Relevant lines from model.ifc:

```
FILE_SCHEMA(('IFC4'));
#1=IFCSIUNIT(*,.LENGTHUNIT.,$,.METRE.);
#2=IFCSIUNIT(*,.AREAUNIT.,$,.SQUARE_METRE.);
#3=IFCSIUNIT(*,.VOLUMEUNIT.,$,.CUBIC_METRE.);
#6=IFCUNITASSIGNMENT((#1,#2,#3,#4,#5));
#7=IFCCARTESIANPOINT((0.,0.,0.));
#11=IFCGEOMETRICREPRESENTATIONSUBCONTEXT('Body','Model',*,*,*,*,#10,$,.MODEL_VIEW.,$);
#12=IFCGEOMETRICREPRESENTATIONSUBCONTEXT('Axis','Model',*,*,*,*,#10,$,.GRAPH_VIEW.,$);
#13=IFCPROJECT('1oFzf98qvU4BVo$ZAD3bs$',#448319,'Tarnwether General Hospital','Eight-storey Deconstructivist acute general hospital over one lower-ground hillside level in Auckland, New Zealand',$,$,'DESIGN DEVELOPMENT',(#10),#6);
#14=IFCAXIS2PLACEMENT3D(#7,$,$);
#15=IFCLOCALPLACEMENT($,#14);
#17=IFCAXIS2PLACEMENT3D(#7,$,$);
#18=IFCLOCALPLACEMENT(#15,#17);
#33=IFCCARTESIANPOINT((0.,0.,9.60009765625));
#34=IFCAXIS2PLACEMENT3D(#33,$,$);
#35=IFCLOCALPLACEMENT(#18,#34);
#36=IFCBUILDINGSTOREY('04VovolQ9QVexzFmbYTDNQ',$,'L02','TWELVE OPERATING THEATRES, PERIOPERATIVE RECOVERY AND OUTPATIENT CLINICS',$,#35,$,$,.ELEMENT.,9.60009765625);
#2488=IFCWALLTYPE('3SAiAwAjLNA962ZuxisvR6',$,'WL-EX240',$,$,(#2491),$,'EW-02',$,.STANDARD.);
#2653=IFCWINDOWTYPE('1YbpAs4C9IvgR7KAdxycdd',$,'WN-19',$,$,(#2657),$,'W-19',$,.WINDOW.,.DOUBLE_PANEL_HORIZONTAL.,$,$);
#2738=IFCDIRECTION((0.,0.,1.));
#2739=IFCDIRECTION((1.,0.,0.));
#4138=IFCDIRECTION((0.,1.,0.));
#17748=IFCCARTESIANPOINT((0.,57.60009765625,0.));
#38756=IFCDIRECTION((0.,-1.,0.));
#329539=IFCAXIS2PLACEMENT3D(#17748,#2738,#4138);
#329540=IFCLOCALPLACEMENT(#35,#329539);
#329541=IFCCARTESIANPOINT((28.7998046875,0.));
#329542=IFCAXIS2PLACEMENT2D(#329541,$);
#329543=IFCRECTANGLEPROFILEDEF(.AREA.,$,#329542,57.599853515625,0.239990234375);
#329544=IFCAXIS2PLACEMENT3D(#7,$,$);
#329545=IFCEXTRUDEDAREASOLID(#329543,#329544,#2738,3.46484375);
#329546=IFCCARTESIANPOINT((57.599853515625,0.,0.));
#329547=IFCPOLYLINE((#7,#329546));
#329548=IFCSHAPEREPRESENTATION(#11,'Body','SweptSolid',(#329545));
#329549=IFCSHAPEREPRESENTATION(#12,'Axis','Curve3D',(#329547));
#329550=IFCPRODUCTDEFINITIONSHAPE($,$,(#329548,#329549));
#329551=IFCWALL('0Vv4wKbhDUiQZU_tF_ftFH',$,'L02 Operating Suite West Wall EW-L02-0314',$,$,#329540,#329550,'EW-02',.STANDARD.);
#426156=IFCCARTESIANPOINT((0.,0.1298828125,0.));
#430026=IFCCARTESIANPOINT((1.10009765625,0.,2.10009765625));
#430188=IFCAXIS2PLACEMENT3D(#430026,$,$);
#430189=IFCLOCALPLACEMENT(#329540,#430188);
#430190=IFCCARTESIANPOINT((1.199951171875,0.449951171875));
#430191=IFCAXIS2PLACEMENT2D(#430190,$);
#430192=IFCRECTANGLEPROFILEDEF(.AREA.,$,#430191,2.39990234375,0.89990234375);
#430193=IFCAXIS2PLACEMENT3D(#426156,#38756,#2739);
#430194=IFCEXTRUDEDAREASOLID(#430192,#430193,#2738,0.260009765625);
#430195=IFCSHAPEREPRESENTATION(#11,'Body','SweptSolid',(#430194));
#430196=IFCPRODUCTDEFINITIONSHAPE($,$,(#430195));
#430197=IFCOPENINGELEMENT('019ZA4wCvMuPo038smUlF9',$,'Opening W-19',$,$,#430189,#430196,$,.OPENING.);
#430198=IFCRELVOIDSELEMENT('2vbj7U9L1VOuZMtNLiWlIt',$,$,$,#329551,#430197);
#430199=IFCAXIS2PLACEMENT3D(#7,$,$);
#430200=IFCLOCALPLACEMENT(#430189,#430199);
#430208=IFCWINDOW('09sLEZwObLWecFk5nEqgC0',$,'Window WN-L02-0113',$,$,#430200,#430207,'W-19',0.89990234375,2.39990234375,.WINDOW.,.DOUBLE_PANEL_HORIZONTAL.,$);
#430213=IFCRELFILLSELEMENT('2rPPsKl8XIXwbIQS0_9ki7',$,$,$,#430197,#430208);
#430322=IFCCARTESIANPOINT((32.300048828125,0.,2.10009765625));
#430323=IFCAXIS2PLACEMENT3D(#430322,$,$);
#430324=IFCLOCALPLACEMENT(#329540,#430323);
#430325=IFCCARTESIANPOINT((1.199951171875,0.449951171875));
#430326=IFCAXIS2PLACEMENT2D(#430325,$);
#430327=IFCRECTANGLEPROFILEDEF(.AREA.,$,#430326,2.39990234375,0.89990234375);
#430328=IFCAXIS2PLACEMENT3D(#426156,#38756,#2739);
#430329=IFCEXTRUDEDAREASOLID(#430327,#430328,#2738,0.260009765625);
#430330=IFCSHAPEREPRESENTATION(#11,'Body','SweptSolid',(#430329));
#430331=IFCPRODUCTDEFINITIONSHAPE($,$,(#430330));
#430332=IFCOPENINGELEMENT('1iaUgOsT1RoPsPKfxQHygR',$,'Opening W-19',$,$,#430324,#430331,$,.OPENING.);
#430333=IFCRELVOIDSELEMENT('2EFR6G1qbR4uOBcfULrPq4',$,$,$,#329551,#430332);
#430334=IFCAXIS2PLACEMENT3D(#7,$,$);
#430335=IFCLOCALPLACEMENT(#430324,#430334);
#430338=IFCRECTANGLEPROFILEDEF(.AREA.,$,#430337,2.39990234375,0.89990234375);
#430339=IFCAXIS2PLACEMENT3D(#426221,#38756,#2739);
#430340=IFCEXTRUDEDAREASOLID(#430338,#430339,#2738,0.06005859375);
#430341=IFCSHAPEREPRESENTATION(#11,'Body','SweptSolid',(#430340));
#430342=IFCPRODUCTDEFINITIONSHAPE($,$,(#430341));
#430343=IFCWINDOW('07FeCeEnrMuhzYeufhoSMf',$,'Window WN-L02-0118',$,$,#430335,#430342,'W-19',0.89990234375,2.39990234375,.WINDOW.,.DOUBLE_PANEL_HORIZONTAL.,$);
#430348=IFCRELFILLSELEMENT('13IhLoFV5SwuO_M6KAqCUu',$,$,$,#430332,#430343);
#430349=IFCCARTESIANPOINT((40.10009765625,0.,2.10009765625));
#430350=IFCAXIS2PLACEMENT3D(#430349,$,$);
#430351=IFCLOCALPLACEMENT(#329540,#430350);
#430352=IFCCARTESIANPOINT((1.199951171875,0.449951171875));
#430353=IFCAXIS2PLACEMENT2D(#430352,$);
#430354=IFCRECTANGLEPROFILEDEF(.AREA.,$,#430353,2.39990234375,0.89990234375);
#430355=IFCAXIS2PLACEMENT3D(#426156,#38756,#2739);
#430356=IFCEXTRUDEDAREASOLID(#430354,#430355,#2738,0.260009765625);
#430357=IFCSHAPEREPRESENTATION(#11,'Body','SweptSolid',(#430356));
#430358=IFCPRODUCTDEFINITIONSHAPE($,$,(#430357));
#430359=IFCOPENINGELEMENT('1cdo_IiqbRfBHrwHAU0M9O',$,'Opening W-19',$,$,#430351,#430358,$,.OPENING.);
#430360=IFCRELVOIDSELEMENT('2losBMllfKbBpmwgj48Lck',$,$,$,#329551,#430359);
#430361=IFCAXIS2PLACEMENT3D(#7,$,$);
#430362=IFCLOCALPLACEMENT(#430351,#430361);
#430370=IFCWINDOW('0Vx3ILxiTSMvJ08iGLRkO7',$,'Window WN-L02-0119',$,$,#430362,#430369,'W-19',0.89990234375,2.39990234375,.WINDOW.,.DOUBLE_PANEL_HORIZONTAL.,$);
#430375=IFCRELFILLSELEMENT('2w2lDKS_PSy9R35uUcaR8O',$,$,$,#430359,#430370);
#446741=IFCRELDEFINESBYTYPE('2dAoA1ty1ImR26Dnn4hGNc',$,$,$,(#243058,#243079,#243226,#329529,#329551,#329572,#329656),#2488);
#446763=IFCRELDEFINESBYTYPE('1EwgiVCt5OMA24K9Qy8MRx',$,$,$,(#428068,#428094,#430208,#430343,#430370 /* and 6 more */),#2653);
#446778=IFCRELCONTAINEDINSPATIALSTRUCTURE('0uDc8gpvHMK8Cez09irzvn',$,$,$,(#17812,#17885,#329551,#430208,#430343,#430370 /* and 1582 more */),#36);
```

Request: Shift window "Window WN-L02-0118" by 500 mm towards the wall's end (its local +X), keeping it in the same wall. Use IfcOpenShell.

```python
import ifcopenshell
import ifcopenshell.api.geometry
import ifcopenshell.util.placement

model = ifcopenshell.open("model.ifc")

window = model.by_id(430343)
opening = window.FillsVoids[0].RelatingOpeningElement
wall = opening.VoidsElements[0].RelatingBuildingElement

wall_matrix = ifcopenshell.util.placement.get_local_placement(wall.ObjectPlacement)
shift = wall_matrix[:3, 0] * 0.5
before = ifcopenshell.util.placement.get_local_placement(window.ObjectPlacement)[:3, 3].copy()

# The window is placed relative to its opening, so it follows when the opening moves.
matrix = ifcopenshell.util.placement.get_local_placement(opening.ObjectPlacement)
matrix[:3, 3] += shift
ifcopenshell.api.geometry.edit_object_placement(
    model, product=opening, matrix=matrix, is_si=False, should_transform_children=True
)

after = ifcopenshell.util.placement.get_local_placement(window.ObjectPlacement)[:3, 3]
print("window moved by", (after - before).round(3) + 0.0)

model.write("model_rev.ifc")
```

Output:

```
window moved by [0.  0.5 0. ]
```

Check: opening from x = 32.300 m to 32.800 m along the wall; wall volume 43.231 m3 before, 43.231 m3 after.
